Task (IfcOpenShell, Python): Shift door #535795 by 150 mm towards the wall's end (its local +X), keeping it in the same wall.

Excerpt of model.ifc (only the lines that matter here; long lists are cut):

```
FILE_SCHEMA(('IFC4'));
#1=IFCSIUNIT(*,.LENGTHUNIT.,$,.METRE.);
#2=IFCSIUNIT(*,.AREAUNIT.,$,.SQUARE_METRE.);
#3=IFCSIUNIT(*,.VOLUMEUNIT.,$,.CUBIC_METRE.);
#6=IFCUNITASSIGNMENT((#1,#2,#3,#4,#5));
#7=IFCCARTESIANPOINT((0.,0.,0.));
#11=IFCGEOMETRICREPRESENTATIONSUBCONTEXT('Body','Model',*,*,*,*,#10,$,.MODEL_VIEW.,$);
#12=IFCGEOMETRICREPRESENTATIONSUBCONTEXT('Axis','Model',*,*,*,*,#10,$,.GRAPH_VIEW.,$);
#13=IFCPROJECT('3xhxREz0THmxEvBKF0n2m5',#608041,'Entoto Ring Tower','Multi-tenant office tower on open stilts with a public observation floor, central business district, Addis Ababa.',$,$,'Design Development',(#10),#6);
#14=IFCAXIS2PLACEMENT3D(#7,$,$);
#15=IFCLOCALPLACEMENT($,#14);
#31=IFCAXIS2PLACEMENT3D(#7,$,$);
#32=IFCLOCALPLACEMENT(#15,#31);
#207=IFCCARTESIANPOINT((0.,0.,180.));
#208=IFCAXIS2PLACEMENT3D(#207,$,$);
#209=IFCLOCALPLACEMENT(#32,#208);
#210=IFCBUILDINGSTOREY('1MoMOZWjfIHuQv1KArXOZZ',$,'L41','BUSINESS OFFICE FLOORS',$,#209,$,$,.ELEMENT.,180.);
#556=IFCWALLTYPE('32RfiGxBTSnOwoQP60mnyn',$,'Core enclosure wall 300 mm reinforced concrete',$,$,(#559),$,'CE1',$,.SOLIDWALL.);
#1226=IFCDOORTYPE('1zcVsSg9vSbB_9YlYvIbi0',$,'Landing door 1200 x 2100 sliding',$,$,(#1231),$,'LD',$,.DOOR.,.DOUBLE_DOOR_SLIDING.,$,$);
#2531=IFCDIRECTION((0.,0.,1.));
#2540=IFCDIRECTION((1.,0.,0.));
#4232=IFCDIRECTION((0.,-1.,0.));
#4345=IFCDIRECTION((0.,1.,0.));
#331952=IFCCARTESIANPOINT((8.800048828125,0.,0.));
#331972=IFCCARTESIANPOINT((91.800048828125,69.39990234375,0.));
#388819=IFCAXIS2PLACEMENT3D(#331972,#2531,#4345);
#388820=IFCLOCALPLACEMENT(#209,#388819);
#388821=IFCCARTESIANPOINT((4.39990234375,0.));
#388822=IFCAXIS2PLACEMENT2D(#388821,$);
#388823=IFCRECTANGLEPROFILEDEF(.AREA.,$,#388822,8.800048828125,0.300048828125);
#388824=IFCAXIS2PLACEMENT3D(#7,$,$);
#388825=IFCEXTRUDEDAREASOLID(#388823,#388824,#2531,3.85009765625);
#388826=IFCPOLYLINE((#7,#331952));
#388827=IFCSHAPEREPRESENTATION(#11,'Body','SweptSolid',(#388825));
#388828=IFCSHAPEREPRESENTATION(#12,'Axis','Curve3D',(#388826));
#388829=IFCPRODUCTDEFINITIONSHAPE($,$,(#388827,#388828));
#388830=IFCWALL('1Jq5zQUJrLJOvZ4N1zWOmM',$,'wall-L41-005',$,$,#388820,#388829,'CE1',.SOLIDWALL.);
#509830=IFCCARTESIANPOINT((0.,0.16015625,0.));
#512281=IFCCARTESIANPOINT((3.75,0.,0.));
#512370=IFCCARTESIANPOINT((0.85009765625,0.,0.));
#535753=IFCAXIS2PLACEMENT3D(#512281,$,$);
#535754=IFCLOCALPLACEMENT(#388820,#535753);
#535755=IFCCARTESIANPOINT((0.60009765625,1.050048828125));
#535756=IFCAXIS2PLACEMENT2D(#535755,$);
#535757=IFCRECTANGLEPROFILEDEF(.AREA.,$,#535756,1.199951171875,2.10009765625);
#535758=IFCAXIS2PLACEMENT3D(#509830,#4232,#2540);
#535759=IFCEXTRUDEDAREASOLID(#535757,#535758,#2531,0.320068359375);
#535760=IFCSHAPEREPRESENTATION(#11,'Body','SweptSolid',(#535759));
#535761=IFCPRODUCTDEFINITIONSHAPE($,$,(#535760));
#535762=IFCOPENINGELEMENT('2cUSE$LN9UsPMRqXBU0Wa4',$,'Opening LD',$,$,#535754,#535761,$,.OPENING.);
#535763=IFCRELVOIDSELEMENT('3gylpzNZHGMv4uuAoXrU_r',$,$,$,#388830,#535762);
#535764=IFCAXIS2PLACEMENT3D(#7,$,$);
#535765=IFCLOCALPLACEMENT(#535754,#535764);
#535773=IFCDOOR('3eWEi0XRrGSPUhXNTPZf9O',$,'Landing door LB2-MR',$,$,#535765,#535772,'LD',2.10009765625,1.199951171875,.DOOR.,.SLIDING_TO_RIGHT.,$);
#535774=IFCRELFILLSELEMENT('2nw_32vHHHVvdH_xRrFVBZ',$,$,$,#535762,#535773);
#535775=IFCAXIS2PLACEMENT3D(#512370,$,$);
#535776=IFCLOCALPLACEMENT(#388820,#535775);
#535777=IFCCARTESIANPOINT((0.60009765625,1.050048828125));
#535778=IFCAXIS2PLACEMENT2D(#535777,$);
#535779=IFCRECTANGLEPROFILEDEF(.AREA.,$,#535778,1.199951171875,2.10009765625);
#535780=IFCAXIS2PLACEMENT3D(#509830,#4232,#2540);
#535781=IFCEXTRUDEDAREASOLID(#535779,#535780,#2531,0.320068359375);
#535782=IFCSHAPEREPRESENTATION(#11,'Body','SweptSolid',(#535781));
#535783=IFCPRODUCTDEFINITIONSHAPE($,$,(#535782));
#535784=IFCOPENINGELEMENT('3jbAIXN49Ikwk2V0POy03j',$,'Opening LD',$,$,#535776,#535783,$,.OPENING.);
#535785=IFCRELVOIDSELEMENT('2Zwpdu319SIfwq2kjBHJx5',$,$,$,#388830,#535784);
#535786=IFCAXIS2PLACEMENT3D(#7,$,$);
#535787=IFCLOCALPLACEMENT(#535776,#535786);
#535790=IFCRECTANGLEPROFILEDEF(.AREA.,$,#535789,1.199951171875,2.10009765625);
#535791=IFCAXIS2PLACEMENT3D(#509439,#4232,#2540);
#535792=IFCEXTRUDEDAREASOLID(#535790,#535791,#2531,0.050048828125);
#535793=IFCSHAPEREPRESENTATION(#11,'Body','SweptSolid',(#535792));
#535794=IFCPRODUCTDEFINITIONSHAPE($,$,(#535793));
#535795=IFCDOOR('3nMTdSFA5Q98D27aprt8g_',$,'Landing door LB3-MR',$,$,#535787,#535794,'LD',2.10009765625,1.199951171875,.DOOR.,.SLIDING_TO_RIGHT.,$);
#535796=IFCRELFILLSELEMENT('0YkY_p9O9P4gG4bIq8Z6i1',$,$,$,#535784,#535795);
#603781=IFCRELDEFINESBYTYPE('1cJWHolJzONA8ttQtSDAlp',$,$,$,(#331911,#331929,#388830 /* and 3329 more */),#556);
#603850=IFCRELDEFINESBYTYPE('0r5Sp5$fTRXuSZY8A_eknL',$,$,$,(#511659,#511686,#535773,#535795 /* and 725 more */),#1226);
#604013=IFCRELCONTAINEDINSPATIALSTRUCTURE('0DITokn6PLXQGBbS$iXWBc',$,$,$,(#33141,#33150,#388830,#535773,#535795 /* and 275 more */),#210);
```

```python
import ifcopenshell
import ifcopenshell.api.geometry
import ifcopenshell.util.placement
import ifcopenshell.util.unit

model = ifcopenshell.open("model.ifc")
unit_scale = ifcopenshell.util.unit.calculate_unit_scale(model)

door = model.by_guid("3nMTdSFA5Q98D27aprt8g_")
opening = door.FillsVoids[0].RelatingOpeningElement
wall = opening.VoidsElements[0].RelatingBuildingElement

wall_matrix = ifcopenshell.util.placement.get_local_placement(wall.ObjectPlacement)
shift = wall_matrix[:3, 0] * 0.15 / unit_scale
before = ifcopenshell.util.placement.get_local_placement(door.ObjectPlacement)[:3, 3].copy()

# The door is placed relative to its opening, so it follows when the opening moves.
matrix = ifcopenshell.util.placement.get_local_placement(opening.ObjectPlacement)
matrix[:3, 3] += shift
ifcopenshell.api.geometry.edit_object_placement(
    model, product=opening, matrix=matrix, is_si=False, should_transform_children=True
)

after = ifcopenshell.util.placement.get_local_placement(door.ObjectPlacement)[:3, 3]
print("door moved by", (after - before).round(3) + 0.0)

model.write("model_updated.ifc")
```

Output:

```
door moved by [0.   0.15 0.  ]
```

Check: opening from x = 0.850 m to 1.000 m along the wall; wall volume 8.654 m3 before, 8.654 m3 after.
